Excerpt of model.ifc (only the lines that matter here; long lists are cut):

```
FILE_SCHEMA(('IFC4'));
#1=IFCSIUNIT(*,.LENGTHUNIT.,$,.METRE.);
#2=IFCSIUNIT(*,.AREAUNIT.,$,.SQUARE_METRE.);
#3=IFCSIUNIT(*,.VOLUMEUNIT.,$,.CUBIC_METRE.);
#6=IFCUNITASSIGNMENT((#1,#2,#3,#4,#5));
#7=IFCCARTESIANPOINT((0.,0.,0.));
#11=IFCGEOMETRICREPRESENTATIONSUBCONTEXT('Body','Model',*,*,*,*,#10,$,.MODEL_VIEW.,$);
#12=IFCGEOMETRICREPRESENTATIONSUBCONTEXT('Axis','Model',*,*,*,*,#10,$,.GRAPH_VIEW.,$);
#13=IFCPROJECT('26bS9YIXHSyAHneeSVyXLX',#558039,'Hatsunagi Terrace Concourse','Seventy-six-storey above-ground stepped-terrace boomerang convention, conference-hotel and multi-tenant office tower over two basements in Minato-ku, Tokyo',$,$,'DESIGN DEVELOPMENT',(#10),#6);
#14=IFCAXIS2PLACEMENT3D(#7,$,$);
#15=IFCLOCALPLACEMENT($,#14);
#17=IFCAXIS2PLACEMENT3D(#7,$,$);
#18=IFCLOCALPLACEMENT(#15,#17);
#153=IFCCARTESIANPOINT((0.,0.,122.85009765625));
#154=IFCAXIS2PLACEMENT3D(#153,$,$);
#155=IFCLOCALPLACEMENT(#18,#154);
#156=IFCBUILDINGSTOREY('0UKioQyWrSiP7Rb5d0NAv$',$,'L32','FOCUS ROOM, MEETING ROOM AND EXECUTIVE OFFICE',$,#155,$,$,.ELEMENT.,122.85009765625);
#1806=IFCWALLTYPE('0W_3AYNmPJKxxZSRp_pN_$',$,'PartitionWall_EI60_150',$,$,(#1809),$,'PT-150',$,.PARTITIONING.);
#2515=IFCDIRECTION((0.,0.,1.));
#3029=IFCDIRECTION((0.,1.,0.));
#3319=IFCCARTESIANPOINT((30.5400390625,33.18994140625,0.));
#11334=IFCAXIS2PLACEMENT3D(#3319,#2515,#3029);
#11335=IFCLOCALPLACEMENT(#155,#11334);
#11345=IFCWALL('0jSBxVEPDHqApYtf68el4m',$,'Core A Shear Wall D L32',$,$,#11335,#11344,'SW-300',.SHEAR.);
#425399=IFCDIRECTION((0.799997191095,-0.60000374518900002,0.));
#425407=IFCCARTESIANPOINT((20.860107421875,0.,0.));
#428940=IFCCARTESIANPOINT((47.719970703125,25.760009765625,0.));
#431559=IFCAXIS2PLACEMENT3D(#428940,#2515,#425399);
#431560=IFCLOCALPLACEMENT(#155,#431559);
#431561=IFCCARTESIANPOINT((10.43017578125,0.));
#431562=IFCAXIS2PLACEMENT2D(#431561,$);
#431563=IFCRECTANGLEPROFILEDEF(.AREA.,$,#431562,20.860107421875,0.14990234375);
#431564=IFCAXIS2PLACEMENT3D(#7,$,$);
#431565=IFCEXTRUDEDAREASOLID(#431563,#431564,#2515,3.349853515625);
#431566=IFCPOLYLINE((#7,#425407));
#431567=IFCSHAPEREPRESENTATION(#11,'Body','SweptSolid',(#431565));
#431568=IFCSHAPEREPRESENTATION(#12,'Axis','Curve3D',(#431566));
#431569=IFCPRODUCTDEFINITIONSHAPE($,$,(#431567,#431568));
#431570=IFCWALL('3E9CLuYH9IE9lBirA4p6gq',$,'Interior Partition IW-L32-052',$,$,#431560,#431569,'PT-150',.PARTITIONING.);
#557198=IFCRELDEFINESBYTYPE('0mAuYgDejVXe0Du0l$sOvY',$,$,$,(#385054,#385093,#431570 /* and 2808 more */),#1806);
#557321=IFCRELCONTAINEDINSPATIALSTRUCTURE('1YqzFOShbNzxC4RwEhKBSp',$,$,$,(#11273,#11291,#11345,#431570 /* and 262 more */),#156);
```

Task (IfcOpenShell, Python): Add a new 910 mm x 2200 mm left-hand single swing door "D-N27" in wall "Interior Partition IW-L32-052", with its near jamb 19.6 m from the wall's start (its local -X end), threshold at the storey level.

```python
import numpy as np
import ifcopenshell
import ifcopenshell.api.feature
import ifcopenshell.api.geometry
import ifcopenshell.api.root
import ifcopenshell.api.spatial
import ifcopenshell.geom
import ifcopenshell.util.element
import ifcopenshell.util.placement
import ifcopenshell.util.representation
import ifcopenshell.util.shape
import ifcopenshell.util.unit

model = ifcopenshell.open("model.ifc")
unit_scale = ifcopenshell.util.unit.calculate_unit_scale(model)
settings = ifcopenshell.geom.settings()


def volume(element):
    """Net volume in cubic metres, openings subtracted."""
    shape = ifcopenshell.geom.create_shape(settings, element)
    return ifcopenshell.util.shape.get_volume(shape.geometry)


wall = model.by_guid("3E9CLuYH9IE9lBirA4p6gq")
storey = ifcopenshell.util.element.get_container(wall, ifc_class="IfcBuildingStorey")
context = ifcopenshell.util.representation.get_context(model, "Model", "Body", "MODEL_VIEW")
before = volume(wall)

width, height, from_end, sill = 0.91, 2.2, 19.6, 0.0  # metres

# The wall runs along its own X axis, and the end named is its -X end.
wall_shape = ifcopenshell.geom.create_shape(settings, wall)
x, y, z = ifcopenshell.util.shape.get_vertices(wall_shape.geometry).T
start = x.min() + from_end
face, thickness = float(y.min()), float(y.max() - y.min())
wall_matrix = ifcopenshell.util.placement.get_local_placement(wall.ObjectPlacement)
level = ifcopenshell.util.placement.get_local_placement(storey.ObjectPlacement)[2, 3]


def in_wall(x, y):
    """Placement at x, y metres in the wall's axes, at sill height."""
    matrix = wall_matrix.copy()
    matrix[:, 3] = wall_matrix @ np.array([x / unit_scale, y / unit_scale, 0.0, 1.0])
    matrix[2, 3] = level + sill / unit_scale
    return matrix


# Opening: a box that overshoots both wall faces by 50 mm.
opening = ifcopenshell.api.root.create_entity(model, ifc_class="IfcOpeningElement", predefined_type="OPENING")
box = ifcopenshell.api.geometry.add_wall_representation(
    model, context=context, length=width, height=height, thickness=thickness + 0.1
)
ifcopenshell.api.geometry.assign_representation(model, product=opening, representation=box)
ifcopenshell.api.geometry.edit_object_placement(model, product=opening, matrix=in_wall(start, face - 0.05), is_si=False)
ifcopenshell.api.feature.add_feature(model, feature=opening, element=wall)

door = ifcopenshell.api.root.create_entity(model, ifc_class="IfcDoor", name="D-N27", predefined_type="DOOR")
door.OverallWidth, door.OverallHeight = width / unit_scale, height / unit_scale
door.OperationType = "SINGLE_SWING_LEFT"
body = ifcopenshell.api.geometry.add_door_representation(
    model,
    context=context,
    overall_width=door.OverallWidth,
    overall_height=door.OverallHeight,
    operation_type="SINGLE_SWING_LEFT",
    lining_properties={"LiningDepth": thickness / unit_scale, "ThresholdDepth": thickness / unit_scale},
)
ifcopenshell.api.geometry.assign_representation(model, product=door, representation=body)
ifcopenshell.api.spatial.assign_container(model, products=[door], relating_structure=storey)
ifcopenshell.api.feature.add_filling(model, opening=opening, element=door)

# The lining spans the wall, so the door starts at the wall face.
ifcopenshell.api.geometry.edit_object_placement(model, product=door, matrix=in_wall(start, face), is_si=False)

after = volume(wall)

print(f"wall volume {before:.3f} -> {after:.3f} m3")

model.write("model_edited.ifc")
```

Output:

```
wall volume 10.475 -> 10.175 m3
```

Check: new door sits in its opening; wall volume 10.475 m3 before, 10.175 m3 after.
